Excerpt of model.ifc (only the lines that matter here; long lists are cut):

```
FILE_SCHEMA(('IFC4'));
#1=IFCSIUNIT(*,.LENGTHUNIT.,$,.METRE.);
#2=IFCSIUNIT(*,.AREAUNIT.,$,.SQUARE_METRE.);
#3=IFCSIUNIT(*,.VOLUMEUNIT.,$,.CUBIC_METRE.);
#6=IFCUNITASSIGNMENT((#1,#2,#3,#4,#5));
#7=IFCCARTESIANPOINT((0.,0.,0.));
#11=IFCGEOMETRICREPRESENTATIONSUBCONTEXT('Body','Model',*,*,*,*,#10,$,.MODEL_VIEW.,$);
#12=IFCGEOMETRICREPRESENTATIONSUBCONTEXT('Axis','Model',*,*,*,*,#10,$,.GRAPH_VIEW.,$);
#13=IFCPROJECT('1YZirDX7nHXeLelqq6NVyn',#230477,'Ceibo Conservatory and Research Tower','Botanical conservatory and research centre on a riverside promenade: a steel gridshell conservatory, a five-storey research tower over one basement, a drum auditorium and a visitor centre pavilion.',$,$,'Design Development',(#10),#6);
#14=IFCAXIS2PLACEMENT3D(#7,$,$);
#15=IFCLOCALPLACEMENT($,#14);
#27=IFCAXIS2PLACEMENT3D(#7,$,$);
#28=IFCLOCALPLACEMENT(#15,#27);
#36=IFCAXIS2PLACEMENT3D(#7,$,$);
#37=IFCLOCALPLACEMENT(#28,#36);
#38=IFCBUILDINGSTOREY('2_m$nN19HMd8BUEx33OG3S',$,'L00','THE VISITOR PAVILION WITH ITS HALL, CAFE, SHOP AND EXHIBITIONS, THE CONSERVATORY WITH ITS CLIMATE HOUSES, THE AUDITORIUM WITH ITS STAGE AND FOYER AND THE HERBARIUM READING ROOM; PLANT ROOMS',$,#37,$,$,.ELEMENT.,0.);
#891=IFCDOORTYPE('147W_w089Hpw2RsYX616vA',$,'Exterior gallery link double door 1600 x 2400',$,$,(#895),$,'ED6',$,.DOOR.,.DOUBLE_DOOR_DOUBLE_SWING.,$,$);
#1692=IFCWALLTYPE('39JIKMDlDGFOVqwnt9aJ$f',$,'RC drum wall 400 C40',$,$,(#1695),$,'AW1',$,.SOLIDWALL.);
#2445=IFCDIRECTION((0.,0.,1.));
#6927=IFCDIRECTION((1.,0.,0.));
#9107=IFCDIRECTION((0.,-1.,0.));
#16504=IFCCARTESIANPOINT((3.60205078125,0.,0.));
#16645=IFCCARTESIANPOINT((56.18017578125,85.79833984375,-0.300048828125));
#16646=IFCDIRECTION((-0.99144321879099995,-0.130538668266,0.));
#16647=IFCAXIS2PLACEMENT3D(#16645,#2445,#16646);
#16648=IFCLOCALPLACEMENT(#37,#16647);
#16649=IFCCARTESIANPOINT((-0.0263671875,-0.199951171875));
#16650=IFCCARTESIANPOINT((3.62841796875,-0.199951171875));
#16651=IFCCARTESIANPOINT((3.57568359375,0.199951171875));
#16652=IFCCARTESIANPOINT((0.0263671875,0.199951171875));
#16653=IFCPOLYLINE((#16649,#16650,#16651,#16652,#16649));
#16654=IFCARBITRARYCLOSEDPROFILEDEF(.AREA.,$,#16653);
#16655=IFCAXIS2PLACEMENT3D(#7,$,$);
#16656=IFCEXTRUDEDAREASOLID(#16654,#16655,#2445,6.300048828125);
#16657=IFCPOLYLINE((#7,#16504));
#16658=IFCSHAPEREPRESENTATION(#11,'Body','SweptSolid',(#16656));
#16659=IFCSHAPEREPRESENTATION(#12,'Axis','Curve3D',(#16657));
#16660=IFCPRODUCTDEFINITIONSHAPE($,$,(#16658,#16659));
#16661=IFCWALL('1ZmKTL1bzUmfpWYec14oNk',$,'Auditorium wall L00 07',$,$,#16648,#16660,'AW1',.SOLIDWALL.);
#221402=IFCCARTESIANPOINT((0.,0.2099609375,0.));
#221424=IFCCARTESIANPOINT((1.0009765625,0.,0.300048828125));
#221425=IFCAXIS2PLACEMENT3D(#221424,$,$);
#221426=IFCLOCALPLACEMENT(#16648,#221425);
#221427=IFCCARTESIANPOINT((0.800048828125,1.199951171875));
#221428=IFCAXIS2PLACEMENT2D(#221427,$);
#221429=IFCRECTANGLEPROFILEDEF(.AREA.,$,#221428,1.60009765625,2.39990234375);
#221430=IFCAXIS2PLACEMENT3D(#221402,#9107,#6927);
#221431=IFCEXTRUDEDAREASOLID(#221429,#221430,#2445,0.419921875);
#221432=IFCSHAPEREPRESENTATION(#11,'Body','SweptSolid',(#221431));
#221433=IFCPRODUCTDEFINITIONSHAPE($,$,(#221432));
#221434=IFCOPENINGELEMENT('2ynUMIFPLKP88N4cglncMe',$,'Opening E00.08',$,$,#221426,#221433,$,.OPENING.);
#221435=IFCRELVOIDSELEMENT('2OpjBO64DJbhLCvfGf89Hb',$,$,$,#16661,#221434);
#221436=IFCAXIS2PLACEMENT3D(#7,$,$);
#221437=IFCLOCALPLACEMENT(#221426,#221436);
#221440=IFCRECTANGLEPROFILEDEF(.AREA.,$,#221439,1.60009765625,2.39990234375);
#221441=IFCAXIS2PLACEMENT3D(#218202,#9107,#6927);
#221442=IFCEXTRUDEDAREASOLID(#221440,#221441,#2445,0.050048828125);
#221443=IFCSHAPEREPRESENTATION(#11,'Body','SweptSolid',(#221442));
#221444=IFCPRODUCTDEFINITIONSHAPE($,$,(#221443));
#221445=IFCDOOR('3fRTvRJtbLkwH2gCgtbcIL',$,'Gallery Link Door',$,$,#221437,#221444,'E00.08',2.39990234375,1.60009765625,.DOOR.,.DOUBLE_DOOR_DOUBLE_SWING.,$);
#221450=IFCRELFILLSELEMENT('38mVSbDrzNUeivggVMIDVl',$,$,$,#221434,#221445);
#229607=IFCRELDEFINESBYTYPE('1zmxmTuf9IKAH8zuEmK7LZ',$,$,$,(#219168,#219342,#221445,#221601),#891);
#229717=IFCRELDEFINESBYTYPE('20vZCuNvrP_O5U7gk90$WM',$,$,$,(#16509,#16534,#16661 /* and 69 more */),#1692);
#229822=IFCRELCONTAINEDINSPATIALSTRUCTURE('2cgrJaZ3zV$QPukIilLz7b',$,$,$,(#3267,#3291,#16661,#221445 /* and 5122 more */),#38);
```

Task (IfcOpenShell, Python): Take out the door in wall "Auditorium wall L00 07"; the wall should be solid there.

```python
import ifcopenshell
import ifcopenshell.api.feature
import ifcopenshell.api.root
import ifcopenshell.geom
import ifcopenshell.util.shape

model = ifcopenshell.open("model.ifc")
settings = ifcopenshell.geom.settings()


def volume(element):
    """Net volume in cubic metres, openings subtracted."""
    shape = ifcopenshell.geom.create_shape(settings, element)
    return ifcopenshell.util.shape.get_volume(shape.geometry)


door = model.by_guid("3fRTvRJtbLkwH2gCgtbcIL")
opening = door.FillsVoids[0].RelatingOpeningElement
wall = opening.VoidsElements[0].RelatingBuildingElement
before = volume(wall)

ifcopenshell.api.root.remove_product(model, product=door)
ifcopenshell.api.feature.remove_feature(model, feature=opening)

after = volume(wall)

print(f"wall volume {before:.3f} -> {after:.3f} m3")

model.write("model_updated.ifc")
```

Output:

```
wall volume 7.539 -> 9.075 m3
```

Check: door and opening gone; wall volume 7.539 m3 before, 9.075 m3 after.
